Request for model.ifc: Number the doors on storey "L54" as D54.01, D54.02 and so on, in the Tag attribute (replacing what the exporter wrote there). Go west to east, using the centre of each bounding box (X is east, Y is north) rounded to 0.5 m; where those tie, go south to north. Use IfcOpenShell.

First a look at what the model holds.

```python
import ifcopenshell
import ifcopenshell.util.element
import ifcopenshell.util.placement

model = ifcopenshell.open("model.ifc")
print(model.schema)
storey = next(s for s in model.by_type("IfcBuildingStorey") if s.Name == "L54")
doors = [e for e in ifcopenshell.util.element.get_decomposition(storey) if e.is_a("IfcDoor")]
for e in sorted(doors, key=lambda e: e.id()):
    origin = ifcopenshell.util.placement.get_local_placement(e.ObjectPlacement)[:3, 3]
    print(e.id(), e.Tag, e.Name, origin.round(2) + 0.0, sep=" | ")
```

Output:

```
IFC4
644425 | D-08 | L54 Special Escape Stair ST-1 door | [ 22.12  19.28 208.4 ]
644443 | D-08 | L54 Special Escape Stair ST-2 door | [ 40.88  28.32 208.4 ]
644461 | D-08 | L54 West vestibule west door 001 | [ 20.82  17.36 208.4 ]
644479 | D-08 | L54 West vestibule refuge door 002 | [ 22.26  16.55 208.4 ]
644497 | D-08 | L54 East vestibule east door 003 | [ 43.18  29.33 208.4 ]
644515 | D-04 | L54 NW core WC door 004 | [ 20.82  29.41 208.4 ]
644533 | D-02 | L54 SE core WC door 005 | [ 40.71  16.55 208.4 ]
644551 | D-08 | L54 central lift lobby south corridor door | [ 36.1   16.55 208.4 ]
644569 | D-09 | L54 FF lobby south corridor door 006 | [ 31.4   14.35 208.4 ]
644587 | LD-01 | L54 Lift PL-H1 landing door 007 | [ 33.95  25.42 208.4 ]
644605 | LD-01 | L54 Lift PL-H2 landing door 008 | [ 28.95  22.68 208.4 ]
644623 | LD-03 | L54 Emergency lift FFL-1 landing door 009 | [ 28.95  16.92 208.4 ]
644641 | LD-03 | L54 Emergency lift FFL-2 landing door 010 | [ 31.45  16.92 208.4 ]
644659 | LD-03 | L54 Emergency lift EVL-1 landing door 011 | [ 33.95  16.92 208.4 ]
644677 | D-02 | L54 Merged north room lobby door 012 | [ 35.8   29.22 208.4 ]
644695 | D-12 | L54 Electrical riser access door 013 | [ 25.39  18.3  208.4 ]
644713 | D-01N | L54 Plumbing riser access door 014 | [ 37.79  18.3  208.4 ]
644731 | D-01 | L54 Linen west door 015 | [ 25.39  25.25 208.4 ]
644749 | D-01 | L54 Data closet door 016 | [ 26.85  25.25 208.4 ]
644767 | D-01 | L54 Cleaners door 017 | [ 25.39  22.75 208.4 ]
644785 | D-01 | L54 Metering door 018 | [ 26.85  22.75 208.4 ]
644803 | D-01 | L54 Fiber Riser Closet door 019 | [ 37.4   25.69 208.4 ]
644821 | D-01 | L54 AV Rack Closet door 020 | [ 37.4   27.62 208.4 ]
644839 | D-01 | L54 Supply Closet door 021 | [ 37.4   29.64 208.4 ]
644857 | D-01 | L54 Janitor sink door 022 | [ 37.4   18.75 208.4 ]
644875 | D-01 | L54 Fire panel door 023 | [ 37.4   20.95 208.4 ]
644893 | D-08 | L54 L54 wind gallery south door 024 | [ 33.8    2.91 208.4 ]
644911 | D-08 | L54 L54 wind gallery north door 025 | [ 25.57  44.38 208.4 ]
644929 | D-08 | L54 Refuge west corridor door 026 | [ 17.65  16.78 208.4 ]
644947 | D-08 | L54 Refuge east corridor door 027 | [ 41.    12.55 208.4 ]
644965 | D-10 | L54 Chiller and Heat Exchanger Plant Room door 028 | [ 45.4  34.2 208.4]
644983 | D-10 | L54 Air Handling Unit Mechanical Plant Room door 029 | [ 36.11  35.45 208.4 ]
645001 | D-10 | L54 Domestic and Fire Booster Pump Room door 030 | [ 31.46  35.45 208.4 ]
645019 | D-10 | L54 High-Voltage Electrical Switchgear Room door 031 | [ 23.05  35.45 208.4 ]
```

```python
import ifcopenshell
import ifcopenshell.geom
import ifcopenshell.util.element
import ifcopenshell.util.shape

model = ifcopenshell.open("model.ifc")
settings = ifcopenshell.geom.settings()
settings.set("use-world-coords", True)


def centre(element):
    shape = ifcopenshell.geom.create_shape(settings, element)
    return ifcopenshell.util.shape.get_bbox_centroid(shape.geometry)


storey = next(s for s in model.by_type("IfcBuildingStorey") if s.Name == "L54")
doors = [e for e in ifcopenshell.util.element.get_decomposition(storey) if e.is_a("IfcDoor")]

# Insertion points can sit at a corner or the storey origin, so sort by the geometry (in metres).
centres = {e: centre(e) for e in doors}
doors.sort(key=lambda e: (round(centres[e][0] / 0.5), centres[e][1]))

for i, e in enumerate(doors, start=1):
    number = f"D54.{i:02d}"
    e.Tag = number
    print(e.id(), number)

model.write("model-out.ifc")
```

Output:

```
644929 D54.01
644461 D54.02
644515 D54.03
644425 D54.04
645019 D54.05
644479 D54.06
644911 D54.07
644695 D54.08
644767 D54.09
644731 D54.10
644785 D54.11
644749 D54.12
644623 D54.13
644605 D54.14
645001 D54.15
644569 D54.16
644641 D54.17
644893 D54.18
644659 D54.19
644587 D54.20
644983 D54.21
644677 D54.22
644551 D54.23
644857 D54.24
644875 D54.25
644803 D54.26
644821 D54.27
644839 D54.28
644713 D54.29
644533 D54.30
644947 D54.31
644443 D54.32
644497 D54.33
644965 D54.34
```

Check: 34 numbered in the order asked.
